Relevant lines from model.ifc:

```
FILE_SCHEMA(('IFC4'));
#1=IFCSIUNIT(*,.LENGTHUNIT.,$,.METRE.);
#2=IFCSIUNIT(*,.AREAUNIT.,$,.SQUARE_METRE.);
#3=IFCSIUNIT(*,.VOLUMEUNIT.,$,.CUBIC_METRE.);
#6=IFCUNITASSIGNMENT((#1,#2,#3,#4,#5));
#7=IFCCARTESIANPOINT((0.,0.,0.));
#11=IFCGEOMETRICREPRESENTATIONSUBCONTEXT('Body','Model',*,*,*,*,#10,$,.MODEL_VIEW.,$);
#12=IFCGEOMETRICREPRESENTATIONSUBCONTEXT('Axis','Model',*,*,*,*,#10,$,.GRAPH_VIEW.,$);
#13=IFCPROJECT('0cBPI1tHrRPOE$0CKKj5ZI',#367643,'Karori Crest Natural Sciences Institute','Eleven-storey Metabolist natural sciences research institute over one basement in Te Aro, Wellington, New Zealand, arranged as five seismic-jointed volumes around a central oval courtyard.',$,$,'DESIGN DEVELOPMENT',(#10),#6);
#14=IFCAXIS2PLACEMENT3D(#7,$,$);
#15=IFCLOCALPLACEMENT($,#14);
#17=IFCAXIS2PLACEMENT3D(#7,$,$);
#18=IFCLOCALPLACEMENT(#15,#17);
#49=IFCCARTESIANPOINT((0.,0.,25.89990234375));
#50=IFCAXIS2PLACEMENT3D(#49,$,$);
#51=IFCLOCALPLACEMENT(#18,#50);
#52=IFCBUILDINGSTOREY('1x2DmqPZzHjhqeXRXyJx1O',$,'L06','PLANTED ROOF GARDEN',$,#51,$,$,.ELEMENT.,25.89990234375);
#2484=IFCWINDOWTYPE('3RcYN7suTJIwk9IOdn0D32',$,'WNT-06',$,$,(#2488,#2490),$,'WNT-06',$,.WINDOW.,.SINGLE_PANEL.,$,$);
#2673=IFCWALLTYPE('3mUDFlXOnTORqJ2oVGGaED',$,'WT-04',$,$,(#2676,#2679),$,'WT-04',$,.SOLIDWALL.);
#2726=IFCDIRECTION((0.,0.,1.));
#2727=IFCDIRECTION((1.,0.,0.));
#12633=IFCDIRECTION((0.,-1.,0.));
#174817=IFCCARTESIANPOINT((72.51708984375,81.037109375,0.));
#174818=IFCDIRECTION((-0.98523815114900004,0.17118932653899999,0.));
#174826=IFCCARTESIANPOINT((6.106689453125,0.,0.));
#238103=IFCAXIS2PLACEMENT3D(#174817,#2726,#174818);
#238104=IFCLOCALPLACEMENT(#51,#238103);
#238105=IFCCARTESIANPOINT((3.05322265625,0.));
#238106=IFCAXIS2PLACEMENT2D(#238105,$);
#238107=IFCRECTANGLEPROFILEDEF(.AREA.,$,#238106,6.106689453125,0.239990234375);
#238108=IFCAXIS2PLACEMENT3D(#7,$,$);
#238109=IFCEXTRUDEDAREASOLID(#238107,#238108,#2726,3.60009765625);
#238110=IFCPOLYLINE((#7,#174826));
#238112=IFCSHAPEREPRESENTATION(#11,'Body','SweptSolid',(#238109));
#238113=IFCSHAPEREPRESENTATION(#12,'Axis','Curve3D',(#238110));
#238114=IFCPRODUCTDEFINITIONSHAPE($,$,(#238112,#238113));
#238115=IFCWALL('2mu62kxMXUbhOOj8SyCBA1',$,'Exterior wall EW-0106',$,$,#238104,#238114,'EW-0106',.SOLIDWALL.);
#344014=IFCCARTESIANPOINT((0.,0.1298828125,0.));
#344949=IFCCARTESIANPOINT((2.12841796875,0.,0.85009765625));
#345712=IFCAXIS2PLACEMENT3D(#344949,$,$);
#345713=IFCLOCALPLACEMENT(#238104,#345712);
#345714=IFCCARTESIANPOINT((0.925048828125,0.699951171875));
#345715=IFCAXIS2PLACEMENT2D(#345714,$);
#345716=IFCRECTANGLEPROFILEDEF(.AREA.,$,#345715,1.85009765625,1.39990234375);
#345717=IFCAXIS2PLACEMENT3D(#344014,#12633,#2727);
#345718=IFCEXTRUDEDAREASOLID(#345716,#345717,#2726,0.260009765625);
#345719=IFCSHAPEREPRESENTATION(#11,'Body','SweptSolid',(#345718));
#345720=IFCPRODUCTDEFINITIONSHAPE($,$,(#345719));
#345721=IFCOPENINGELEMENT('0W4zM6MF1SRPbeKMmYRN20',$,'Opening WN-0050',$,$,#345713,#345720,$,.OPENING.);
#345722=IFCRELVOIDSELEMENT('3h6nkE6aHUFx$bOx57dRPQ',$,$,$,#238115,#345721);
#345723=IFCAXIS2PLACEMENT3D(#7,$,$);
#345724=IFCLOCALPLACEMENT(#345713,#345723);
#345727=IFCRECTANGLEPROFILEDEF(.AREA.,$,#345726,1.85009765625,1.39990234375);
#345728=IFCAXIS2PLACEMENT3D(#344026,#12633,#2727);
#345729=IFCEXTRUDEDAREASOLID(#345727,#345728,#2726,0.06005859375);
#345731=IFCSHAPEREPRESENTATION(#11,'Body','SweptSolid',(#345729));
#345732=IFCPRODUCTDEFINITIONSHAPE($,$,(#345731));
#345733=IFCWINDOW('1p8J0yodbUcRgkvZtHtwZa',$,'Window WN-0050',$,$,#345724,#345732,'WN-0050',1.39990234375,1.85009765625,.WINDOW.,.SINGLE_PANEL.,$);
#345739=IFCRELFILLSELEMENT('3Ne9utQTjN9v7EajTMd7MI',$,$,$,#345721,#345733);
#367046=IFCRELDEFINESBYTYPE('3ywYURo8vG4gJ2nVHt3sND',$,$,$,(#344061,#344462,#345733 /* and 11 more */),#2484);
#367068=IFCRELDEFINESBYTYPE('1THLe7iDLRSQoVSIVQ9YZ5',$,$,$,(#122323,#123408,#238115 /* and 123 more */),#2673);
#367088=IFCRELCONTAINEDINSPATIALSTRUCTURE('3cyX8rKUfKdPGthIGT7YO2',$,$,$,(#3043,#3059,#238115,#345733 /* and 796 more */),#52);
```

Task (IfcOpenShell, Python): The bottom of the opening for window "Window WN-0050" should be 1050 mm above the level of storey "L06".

```python
import numpy as np
import ifcopenshell
import ifcopenshell.api.geometry
import ifcopenshell.geom
import ifcopenshell.util.element
import ifcopenshell.util.placement
import ifcopenshell.util.shape
import ifcopenshell.util.unit

model = ifcopenshell.open("model.ifc")
unit_scale = ifcopenshell.util.unit.calculate_unit_scale(model)

window = model.by_guid("1p8J0yodbUcRgkvZtHtwZa")
opening = window.FillsVoids[0].RelatingOpeningElement
storey = ifcopenshell.util.element.get_container(window, ifc_class="IfcBuildingStorey")
level = ifcopenshell.util.placement.get_local_placement(storey.ObjectPlacement)[2, 3]

# The opening's origin need not be at the sill, so measure its lowest point.
shape = ifcopenshell.geom.create_shape(ifcopenshell.geom.settings(), opening)
bottom = ifcopenshell.util.shape.get_shape_bottom_elevation(shape, shape.geometry) / unit_scale
dz = level + 1.05 / unit_scale - bottom

shift = np.array([0.0, 0.0, dz])
# The window is placed relative to its opening, so it follows when the opening moves.
matrix = ifcopenshell.util.placement.get_local_placement(opening.ObjectPlacement)
matrix[:3, 3] += shift
ifcopenshell.api.geometry.edit_object_placement(
    model, product=opening, matrix=matrix, is_si=False, should_transform_children=True
)

print(f"moved by {dz * unit_scale:+.3f} m")

model.write("model-out.ifc")
```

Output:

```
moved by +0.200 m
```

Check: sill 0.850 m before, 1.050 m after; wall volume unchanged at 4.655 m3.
